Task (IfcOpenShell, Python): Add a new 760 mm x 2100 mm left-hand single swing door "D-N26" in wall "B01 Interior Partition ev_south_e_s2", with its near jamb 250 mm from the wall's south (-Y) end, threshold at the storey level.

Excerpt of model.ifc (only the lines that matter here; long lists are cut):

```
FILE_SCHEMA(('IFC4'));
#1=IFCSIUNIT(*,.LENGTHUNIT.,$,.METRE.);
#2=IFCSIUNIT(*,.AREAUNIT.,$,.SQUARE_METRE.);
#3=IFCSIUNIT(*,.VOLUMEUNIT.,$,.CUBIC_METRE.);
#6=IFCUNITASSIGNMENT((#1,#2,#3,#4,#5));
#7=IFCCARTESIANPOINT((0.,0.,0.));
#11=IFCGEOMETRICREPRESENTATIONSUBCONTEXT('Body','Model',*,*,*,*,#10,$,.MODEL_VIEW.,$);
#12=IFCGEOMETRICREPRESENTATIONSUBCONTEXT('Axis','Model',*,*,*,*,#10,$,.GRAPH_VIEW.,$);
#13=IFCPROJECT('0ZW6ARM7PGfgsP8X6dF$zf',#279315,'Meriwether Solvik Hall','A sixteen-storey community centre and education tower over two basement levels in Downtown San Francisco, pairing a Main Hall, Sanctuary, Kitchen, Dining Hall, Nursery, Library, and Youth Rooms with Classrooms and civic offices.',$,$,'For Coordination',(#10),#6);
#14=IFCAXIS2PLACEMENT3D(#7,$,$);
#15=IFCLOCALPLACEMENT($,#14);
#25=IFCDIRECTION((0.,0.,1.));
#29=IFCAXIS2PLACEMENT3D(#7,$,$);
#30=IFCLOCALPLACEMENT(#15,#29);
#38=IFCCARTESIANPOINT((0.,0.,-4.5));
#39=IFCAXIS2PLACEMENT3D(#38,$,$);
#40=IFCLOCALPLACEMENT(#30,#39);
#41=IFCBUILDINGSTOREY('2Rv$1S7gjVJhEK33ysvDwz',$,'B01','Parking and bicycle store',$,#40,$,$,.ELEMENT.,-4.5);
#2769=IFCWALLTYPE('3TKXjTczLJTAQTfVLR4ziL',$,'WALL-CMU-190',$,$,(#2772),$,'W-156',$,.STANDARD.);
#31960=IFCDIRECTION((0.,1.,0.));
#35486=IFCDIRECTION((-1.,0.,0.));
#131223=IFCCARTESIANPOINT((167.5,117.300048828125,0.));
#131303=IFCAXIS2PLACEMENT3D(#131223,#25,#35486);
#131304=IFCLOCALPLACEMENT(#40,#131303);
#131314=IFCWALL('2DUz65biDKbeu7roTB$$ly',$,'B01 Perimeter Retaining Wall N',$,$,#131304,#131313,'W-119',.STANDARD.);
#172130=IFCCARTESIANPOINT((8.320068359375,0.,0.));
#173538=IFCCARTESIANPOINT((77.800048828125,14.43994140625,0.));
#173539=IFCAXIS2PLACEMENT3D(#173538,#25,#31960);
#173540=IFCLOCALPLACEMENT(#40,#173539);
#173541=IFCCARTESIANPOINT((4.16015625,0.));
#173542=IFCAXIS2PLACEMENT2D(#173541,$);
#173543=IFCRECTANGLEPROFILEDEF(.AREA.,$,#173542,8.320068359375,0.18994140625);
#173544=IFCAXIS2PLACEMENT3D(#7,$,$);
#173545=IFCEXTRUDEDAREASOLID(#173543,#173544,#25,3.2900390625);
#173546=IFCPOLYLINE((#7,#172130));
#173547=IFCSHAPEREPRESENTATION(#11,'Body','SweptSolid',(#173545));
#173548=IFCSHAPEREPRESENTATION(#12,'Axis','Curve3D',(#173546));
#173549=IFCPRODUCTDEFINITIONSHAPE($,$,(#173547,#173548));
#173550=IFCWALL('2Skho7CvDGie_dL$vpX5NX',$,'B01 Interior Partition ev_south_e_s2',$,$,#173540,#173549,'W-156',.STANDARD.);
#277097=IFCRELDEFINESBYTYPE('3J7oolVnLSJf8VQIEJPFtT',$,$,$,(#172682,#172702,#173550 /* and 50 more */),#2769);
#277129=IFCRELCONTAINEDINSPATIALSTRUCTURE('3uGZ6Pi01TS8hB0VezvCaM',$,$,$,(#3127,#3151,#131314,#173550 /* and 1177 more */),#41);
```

```python
import numpy as np
import ifcopenshell
import ifcopenshell.api.feature
import ifcopenshell.api.geometry
import ifcopenshell.api.root
import ifcopenshell.api.spatial
import ifcopenshell.geom
import ifcopenshell.util.element
import ifcopenshell.util.placement
import ifcopenshell.util.representation
import ifcopenshell.util.shape
import ifcopenshell.util.unit

model = ifcopenshell.open("model.ifc")
unit_scale = ifcopenshell.util.unit.calculate_unit_scale(model)
settings = ifcopenshell.geom.settings()


def volume(element):
    """Net volume in cubic metres, openings subtracted."""
    shape = ifcopenshell.geom.create_shape(settings, element)
    return ifcopenshell.util.shape.get_volume(shape.geometry)


wall = model.by_guid("2Skho7CvDGie_dL$vpX5NX")
storey = ifcopenshell.util.element.get_container(wall, ifc_class="IfcBuildingStorey")
context = ifcopenshell.util.representation.get_context(model, "Model", "Body", "MODEL_VIEW")
before = volume(wall)

width, height, from_end, sill = 0.76, 2.1, 0.25, 0.0  # metres

# The wall runs along its own X axis, and the end named is its -X end.
wall_shape = ifcopenshell.geom.create_shape(settings, wall)
x, y, z = ifcopenshell.util.shape.get_vertices(wall_shape.geometry).T
start = x.min() + from_end
face, thickness = float(y.min()), float(y.max() - y.min())
wall_matrix = ifcopenshell.util.placement.get_local_placement(wall.ObjectPlacement)
level = ifcopenshell.util.placement.get_local_placement(storey.ObjectPlacement)[2, 3]


def in_wall(x, y):
    """Placement at x, y metres in the wall's axes, at sill height."""
    matrix = wall_matrix.copy()
    matrix[:, 3] = wall_matrix @ np.array([x / unit_scale, y / unit_scale, 0.0, 1.0])
    matrix[2, 3] = level + sill / unit_scale
    return matrix


# Opening: a box that overshoots both wall faces by 50 mm.
opening = ifcopenshell.api.root.create_entity(model, ifc_class="IfcOpeningElement", predefined_type="OPENING")
box = ifcopenshell.api.geometry.add_wall_representation(
    model, context=context, length=width, height=height, thickness=thickness + 0.1
)
ifcopenshell.api.geometry.assign_representation(model, product=opening, representation=box)
ifcopenshell.api.geometry.edit_object_placement(model, product=opening, matrix=in_wall(start, face - 0.05), is_si=False)
ifcopenshell.api.feature.add_feature(model, feature=opening, element=wall)

door = ifcopenshell.api.root.create_entity(model, ifc_class="IfcDoor", name="D-N26", predefined_type="DOOR")
door.OverallWidth, door.OverallHeight = width / unit_scale, height / unit_scale
door.OperationType = "SINGLE_SWING_LEFT"
body = ifcopenshell.api.geometry.add_door_representation(
    model,
    context=context,
    overall_width=door.OverallWidth,
    overall_height=door.OverallHeight,
    operation_type="SINGLE_SWING_LEFT",
    lining_properties={"LiningDepth": thickness / unit_scale, "ThresholdDepth": thickness / unit_scale},
)
ifcopenshell.api.geometry.assign_representation(model, product=door, representation=body)
ifcopenshell.api.spatial.assign_container(model, products=[door], relating_structure=storey)
ifcopenshell.api.feature.add_filling(model, opening=opening, element=door)

# The lining spans the wall, so the door starts at the wall face.
ifcopenshell.api.geometry.edit_object_placement(model, product=door, matrix=in_wall(start, face), is_si=False)

after = volume(wall)

print(f"wall volume {before:.3f} -> {after:.3f} m3")

model.write("model_v2.ifc")
```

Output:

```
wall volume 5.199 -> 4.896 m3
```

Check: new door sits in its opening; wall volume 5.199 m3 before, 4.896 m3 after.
